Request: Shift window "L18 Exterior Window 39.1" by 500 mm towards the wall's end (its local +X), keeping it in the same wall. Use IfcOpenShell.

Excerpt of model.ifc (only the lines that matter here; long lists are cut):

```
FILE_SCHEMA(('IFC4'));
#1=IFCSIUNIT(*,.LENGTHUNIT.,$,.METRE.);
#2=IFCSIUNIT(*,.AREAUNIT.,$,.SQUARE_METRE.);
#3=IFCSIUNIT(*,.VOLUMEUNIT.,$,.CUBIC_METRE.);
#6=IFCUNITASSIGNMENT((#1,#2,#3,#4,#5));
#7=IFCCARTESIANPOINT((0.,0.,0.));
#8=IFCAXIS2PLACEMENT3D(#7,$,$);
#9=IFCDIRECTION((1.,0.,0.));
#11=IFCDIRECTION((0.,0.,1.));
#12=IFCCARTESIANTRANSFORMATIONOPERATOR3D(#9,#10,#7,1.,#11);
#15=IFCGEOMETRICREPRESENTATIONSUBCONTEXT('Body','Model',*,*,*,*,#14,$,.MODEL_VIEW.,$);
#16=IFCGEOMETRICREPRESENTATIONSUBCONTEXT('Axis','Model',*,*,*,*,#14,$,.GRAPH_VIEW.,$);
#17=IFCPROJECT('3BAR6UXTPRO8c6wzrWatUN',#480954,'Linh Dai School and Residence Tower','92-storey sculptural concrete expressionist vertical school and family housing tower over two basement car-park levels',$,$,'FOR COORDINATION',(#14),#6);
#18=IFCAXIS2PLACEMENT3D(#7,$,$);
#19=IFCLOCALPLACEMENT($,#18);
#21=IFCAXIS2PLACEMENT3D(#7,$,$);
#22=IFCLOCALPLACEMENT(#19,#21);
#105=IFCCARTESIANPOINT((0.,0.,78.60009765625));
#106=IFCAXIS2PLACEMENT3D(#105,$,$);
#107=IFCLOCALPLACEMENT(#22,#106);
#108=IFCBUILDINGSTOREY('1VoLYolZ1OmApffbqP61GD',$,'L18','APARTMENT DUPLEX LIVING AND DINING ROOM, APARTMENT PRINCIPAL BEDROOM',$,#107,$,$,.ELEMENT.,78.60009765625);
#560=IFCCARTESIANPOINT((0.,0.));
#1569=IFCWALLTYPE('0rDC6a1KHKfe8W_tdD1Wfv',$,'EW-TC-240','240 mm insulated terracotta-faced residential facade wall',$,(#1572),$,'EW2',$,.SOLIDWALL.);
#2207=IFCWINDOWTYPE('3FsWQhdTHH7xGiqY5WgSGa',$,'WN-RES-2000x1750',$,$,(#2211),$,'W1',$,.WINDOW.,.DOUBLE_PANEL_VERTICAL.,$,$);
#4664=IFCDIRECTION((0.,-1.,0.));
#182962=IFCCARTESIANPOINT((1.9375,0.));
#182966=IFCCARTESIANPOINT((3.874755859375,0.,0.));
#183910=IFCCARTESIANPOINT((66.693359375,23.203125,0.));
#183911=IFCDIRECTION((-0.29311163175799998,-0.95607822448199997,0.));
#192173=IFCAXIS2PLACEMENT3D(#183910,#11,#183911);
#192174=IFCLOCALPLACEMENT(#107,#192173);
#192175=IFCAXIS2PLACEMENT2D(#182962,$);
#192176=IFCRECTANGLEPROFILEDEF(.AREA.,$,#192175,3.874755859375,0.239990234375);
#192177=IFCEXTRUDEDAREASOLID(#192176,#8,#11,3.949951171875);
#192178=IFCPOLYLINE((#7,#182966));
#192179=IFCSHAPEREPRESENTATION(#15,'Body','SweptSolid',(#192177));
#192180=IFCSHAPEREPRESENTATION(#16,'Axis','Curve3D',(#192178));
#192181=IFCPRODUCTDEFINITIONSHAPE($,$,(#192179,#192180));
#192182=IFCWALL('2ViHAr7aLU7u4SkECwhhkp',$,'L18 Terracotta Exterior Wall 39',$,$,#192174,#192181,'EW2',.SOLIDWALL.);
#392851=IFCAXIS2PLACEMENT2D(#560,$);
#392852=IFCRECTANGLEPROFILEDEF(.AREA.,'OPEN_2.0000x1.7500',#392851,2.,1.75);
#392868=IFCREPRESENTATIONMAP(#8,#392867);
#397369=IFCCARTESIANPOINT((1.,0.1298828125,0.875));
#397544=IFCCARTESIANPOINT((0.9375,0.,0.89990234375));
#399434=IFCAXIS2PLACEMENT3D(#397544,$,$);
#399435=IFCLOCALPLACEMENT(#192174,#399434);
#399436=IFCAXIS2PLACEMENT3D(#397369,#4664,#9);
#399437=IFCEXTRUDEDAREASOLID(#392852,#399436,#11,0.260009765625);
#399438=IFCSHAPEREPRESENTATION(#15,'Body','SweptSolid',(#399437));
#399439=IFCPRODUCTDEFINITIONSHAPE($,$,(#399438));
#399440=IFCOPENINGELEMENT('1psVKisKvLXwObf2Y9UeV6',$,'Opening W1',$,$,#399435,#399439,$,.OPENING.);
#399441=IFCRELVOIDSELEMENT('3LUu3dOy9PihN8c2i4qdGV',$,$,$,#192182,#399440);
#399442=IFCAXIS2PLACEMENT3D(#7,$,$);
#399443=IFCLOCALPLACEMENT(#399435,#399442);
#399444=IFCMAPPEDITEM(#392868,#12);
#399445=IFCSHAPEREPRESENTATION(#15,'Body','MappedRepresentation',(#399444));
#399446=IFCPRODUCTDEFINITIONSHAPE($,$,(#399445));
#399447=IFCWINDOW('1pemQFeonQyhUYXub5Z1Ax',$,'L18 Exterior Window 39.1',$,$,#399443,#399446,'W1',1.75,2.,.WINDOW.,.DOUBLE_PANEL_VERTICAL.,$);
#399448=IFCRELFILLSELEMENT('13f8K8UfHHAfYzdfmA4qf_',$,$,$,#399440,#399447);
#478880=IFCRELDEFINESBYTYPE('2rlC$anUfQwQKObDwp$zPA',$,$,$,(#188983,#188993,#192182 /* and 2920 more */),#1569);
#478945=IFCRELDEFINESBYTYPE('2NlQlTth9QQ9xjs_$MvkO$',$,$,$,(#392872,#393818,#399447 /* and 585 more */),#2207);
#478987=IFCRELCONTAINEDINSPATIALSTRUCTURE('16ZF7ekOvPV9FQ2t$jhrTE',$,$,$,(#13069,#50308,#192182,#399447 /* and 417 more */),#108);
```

```python
import ifcopenshell
import ifcopenshell.api.geometry
import ifcopenshell.util.placement
import ifcopenshell.util.unit

model = ifcopenshell.open("model.ifc")
unit_scale = ifcopenshell.util.unit.calculate_unit_scale(model)

window = model.by_guid("1pemQFeonQyhUYXub5Z1Ax")
opening = window.FillsVoids[0].RelatingOpeningElement
wall = opening.VoidsElements[0].RelatingBuildingElement

wall_matrix = ifcopenshell.util.placement.get_local_placement(wall.ObjectPlacement)
shift = wall_matrix[:3, 0] * 0.5 / unit_scale
before = ifcopenshell.util.placement.get_local_placement(window.ObjectPlacement)[:3, 3].copy()

# The window is placed relative to its opening, so it follows when the opening moves.
matrix = ifcopenshell.util.placement.get_local_placement(opening.ObjectPlacement)
matrix[:3, 3] += shift
ifcopenshell.api.geometry.edit_object_placement(
    model, product=opening, matrix=matrix, is_si=False, should_transform_children=True
)

after = ifcopenshell.util.placement.get_local_placement(window.ObjectPlacement)[:3, 3]
print("window moved by", (after - before).round(3) + 0.0)

model.write("model_v2.ifc")
```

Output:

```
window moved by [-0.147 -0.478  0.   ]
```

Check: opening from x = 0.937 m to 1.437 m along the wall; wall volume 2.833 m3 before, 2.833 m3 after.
